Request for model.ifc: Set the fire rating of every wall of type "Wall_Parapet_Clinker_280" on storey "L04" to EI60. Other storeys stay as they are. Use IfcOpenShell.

First a look at what the model holds.

```python
import ifcopenshell
import ifcopenshell.util.element

model = ifcopenshell.open("model.ifc")
print(model.schema)
storey = next(s for s in model.by_type("IfcBuildingStorey") if s.Name == "L04")
walls = [e for e in ifcopenshell.util.element.get_decomposition(storey) if e.is_a("IfcWall")]
seen = {}
for e in walls:
    element_type = ifcopenshell.util.element.get_type(e)
    key = (element_type.Name if element_type != e and element_type else None, ifcopenshell.util.element.get_pset(e, "Pset_WallCommon", "FireRating"))
    seen[key] = seen.get(key, 0) + 1
for (name, value), count in sorted(seen.items(), key=str):
    print(count, "x", name, "|", value)
```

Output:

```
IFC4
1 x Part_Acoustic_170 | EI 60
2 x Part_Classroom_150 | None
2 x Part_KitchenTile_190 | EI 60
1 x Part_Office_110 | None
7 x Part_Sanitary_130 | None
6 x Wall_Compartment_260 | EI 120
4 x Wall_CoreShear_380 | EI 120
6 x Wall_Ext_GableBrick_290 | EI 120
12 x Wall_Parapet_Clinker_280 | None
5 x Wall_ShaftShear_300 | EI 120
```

```python
import ifcopenshell
import ifcopenshell.api.pset
import ifcopenshell.util.element

model = ifcopenshell.open("model.ifc")

storey = next(s for s in model.by_type("IfcBuildingStorey") if s.Name == "L04")
walls = [e for e in ifcopenshell.util.element.get_decomposition(storey) if e.is_a("IfcWall")]

count = 0
for e in walls:
    element_type = ifcopenshell.util.element.get_type(e)
    if element_type in (None, e) or element_type.Name != "Wall_Parapet_Clinker_280":
        continue
    # add_pset returns the element's existing set when there is one.
    pset = ifcopenshell.api.pset.add_pset(model, product=e, name="Pset_WallCommon")
    ifcopenshell.api.pset.edit_pset(model, pset=pset, properties={"FireRating": "EI60"})
    count += 1

print(count, "walls updated")

model.write("model_edited.ifc")
```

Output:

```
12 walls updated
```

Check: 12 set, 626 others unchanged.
